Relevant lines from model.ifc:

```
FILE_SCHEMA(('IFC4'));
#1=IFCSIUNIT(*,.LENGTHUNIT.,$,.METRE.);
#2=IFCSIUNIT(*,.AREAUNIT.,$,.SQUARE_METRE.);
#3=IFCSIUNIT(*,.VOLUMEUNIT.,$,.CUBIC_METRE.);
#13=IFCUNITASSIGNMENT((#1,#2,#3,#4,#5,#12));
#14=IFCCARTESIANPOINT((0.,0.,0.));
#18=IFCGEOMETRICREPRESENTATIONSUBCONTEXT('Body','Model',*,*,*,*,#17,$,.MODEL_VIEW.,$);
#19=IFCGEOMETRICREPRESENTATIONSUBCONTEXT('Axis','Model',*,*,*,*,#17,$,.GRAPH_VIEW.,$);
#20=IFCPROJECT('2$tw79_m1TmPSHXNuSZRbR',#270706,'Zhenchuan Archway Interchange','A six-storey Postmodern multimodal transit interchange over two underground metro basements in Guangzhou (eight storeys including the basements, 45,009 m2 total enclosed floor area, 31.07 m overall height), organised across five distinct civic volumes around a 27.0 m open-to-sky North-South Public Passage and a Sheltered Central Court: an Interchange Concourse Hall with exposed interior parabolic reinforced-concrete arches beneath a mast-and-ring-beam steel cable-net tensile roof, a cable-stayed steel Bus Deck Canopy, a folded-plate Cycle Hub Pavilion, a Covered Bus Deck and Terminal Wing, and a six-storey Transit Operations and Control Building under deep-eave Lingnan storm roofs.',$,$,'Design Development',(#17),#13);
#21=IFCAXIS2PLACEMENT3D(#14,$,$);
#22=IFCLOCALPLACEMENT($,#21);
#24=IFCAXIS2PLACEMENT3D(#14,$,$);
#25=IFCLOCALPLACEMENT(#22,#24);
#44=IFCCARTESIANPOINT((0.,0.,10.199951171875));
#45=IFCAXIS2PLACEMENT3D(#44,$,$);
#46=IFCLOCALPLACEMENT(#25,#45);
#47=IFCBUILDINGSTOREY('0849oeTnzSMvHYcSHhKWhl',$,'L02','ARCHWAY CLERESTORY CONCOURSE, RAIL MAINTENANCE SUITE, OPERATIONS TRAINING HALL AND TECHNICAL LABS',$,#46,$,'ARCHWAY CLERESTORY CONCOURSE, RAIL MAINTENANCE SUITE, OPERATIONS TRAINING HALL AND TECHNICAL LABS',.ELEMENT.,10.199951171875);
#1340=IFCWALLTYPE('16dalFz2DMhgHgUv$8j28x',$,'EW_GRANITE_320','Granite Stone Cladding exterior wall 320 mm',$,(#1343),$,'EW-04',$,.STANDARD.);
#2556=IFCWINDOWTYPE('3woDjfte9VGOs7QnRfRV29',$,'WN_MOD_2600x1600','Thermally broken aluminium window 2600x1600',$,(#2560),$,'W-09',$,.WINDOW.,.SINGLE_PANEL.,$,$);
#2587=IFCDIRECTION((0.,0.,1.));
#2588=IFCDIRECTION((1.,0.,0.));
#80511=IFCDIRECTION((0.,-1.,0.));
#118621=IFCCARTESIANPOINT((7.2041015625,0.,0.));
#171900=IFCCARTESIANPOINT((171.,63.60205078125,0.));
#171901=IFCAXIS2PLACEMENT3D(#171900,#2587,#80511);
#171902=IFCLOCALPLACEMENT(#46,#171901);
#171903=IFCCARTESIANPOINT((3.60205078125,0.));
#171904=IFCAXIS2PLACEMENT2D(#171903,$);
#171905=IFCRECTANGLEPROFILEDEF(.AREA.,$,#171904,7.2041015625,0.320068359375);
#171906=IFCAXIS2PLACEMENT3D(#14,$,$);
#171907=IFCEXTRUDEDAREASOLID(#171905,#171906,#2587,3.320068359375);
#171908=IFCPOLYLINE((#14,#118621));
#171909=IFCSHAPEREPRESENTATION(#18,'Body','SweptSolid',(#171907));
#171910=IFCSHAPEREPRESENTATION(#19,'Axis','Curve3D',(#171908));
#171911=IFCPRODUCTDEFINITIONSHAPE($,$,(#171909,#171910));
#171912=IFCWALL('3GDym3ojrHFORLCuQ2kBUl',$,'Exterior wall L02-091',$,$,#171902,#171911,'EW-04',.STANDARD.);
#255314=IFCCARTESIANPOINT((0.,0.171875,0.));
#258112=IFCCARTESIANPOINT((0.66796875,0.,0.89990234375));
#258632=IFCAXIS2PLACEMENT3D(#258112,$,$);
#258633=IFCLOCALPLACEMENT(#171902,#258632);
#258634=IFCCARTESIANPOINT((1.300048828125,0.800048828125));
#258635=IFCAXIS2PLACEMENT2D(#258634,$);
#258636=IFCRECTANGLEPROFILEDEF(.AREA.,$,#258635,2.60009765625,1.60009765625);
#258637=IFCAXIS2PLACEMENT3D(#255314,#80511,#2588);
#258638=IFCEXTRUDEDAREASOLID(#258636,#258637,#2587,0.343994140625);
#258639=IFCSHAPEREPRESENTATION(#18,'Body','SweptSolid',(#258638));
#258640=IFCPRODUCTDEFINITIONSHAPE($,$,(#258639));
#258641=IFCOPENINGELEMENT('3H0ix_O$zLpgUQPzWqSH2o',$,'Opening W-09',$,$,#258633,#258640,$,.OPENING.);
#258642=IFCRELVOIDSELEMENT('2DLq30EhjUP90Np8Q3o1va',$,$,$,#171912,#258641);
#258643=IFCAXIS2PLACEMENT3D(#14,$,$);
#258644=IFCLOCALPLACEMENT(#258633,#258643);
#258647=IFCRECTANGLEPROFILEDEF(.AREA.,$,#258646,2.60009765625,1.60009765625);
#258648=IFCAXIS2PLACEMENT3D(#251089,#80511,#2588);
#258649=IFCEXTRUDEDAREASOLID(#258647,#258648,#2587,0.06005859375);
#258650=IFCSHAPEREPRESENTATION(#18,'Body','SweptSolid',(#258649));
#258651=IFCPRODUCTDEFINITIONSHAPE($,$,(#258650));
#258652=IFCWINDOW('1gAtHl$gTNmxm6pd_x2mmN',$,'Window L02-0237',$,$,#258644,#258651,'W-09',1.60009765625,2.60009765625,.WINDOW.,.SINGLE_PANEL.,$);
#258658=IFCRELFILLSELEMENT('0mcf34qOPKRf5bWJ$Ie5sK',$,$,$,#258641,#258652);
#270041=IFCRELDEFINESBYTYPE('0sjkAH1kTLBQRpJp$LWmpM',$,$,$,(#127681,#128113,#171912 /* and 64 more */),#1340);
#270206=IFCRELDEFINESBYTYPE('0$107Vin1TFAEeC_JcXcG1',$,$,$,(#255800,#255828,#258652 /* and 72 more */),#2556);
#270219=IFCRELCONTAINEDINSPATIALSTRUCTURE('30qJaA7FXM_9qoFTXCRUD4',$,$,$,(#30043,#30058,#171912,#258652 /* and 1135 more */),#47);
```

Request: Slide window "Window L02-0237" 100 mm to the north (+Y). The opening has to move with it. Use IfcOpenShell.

```python
import ifcopenshell
import ifcopenshell.api.geometry
import ifcopenshell.util.placement

model = ifcopenshell.open("model.ifc")

window = model.by_guid("1gAtHl$gTNmxm6pd_x2mmN")
opening = window.FillsVoids[0].RelatingOpeningElement
wall = opening.VoidsElements[0].RelatingBuildingElement

wall_matrix = ifcopenshell.util.placement.get_local_placement(wall.ObjectPlacement)
shift = wall_matrix[:3, 0] * -0.1
before = ifcopenshell.util.placement.get_local_placement(window.ObjectPlacement)[:3, 3].copy()

# The window is placed relative to its opening, so it follows when the opening moves.
matrix = ifcopenshell.util.placement.get_local_placement(opening.ObjectPlacement)
matrix[:3, 3] += shift
ifcopenshell.api.geometry.edit_object_placement(
    model, product=opening, matrix=matrix, is_si=False, should_transform_children=True
)

after = ifcopenshell.util.placement.get_local_placement(window.ObjectPlacement)[:3, 3]
print("window moved by", (after - before).round(3) + 0.0)

model.write("model_v2.ifc")
```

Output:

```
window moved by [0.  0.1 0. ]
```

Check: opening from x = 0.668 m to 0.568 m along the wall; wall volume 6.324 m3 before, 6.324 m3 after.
